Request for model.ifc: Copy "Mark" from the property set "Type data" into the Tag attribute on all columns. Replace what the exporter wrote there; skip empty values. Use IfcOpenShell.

First a look at what the model holds.

```python
import ifcopenshell
import ifcopenshell.util.element

model = ifcopenshell.open("model.ifc")
print(model.schema)
columns = model.by_type("IfcColumn")
print(len(columns), "columns")
for e in columns[:8]:
    source = ifcopenshell.util.element.get_pset(e, "Type data", "Mark")
    target = e.Tag
    print(e.id(), repr(source), repr(target), sep=" | ")
```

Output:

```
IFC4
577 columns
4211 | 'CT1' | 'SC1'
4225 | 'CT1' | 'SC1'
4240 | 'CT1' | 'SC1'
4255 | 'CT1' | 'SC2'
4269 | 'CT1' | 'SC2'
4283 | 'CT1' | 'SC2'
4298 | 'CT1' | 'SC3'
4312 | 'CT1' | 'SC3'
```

```python
import ifcopenshell
import ifcopenshell.util.element

model = ifcopenshell.open("model.ifc")

count = 0
for e in model.by_type("IfcColumn"):
    value = ifcopenshell.util.element.get_pset(e, "Type data", "Mark")
    current = e.Tag
    if not value or not value.strip() or current == value:
        continue
    e.Tag = value
    count += 1

print(count, "columns updated")

model.write("model_edited.ifc")
```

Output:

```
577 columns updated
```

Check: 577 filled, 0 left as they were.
